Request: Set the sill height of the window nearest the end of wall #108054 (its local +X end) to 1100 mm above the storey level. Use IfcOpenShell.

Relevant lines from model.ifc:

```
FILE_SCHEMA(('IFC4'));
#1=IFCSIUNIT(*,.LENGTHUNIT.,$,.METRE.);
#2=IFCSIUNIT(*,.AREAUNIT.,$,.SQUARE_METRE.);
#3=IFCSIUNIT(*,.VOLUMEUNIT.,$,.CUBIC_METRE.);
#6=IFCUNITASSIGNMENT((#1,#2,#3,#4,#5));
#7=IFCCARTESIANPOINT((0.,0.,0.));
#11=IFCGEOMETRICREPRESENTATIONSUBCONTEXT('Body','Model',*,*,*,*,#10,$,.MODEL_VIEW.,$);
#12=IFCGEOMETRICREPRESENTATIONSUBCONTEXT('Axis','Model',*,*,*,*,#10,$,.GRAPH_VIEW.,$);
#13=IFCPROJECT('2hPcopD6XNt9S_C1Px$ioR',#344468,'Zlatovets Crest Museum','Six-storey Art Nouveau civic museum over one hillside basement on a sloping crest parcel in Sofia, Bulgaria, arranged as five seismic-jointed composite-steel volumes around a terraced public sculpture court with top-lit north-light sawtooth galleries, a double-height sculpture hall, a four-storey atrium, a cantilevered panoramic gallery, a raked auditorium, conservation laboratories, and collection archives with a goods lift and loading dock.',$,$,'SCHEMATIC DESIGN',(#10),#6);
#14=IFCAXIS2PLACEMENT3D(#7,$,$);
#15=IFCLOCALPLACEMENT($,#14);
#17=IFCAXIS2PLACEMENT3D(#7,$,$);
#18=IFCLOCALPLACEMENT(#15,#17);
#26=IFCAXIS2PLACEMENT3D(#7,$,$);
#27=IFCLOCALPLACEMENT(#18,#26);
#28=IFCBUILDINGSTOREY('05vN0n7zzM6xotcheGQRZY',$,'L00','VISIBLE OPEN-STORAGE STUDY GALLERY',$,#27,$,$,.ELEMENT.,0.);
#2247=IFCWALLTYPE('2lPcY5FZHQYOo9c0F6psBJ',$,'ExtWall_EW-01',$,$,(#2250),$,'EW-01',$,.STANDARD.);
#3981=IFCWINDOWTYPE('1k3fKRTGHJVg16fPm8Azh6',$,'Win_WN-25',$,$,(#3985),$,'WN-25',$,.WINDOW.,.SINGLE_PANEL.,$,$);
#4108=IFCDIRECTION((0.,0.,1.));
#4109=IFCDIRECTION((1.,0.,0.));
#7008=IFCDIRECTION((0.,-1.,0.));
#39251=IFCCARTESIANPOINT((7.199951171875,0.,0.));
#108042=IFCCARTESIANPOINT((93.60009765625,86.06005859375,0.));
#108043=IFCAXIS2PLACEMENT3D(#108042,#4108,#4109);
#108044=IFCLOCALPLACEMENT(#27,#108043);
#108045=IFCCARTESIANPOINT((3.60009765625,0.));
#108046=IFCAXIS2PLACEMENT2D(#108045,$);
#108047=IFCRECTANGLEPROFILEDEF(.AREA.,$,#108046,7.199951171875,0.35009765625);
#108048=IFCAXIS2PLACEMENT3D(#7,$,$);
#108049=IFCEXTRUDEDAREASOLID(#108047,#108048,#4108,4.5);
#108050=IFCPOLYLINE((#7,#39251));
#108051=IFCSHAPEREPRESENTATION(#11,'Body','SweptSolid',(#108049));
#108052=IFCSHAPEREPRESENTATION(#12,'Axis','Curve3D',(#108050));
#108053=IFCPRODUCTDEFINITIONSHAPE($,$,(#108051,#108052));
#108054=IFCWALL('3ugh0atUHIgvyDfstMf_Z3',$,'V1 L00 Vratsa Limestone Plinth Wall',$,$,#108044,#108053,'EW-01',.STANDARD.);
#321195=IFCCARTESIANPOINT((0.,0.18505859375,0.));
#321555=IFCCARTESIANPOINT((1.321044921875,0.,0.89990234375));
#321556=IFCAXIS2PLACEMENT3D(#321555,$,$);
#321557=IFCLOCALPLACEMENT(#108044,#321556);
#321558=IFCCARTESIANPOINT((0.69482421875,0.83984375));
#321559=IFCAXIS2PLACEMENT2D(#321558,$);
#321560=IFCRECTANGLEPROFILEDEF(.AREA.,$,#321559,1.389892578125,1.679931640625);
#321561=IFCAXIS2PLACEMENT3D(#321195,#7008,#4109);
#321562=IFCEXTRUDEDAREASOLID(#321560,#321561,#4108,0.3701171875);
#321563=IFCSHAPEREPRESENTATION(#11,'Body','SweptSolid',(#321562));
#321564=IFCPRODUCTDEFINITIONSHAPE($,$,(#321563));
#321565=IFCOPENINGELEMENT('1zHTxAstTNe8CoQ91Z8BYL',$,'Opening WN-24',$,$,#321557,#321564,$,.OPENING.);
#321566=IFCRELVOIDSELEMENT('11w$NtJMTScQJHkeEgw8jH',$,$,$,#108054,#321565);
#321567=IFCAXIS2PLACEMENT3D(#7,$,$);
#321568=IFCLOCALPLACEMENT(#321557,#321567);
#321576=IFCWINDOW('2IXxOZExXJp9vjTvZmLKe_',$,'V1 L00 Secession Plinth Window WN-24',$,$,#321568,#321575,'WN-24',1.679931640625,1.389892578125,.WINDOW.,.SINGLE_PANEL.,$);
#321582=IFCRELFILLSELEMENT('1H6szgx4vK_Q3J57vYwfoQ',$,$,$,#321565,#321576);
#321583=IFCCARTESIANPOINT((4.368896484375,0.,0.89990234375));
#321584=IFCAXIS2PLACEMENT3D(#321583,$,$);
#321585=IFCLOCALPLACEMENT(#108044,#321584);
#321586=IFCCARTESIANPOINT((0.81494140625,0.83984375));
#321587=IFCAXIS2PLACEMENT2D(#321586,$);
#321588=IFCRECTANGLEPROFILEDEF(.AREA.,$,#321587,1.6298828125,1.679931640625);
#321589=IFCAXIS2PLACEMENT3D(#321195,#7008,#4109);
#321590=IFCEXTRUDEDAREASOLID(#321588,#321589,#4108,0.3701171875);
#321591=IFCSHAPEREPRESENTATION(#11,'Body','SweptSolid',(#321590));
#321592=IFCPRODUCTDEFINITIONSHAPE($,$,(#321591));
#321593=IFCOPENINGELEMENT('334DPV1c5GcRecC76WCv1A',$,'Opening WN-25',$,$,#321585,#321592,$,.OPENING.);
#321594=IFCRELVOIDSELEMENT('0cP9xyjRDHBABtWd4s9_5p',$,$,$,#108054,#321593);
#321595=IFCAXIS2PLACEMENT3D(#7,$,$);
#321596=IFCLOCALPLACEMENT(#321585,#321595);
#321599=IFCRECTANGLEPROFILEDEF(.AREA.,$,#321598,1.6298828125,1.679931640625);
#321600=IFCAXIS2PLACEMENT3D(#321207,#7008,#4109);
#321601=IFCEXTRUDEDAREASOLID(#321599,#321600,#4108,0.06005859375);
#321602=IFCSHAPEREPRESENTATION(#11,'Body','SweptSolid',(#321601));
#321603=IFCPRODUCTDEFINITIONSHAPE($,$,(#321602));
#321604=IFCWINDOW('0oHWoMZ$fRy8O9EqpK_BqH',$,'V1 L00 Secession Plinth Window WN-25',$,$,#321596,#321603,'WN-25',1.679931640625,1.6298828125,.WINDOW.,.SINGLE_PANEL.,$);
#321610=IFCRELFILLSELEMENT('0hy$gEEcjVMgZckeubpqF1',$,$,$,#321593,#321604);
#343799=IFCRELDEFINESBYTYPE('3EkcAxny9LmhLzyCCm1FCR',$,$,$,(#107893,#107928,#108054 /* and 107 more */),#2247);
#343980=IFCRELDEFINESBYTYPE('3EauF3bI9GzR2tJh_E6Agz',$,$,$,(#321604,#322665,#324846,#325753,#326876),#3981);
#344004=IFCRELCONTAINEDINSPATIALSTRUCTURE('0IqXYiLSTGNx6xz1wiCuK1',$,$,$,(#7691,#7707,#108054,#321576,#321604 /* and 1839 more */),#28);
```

```python
import numpy as np
import ifcopenshell
import ifcopenshell.api.geometry
import ifcopenshell.geom
import ifcopenshell.util.element
import ifcopenshell.util.placement
import ifcopenshell.util.shape
import ifcopenshell.util.unit

model = ifcopenshell.open("model.ifc")
unit_scale = ifcopenshell.util.unit.calculate_unit_scale(model)

window = model.by_id(321604)
opening = window.FillsVoids[0].RelatingOpeningElement
storey = ifcopenshell.util.element.get_container(window, ifc_class="IfcBuildingStorey")
level = ifcopenshell.util.placement.get_local_placement(storey.ObjectPlacement)[2, 3]

# The opening's origin need not be at the sill, so measure its lowest point.
shape = ifcopenshell.geom.create_shape(ifcopenshell.geom.settings(), opening)
bottom = ifcopenshell.util.shape.get_shape_bottom_elevation(shape, shape.geometry) / unit_scale
dz = level + 1.1 - bottom

shift = np.array([0.0, 0.0, dz])
# The window is placed relative to its opening, so it follows when the opening moves.
matrix = ifcopenshell.util.placement.get_local_placement(opening.ObjectPlacement)
matrix[:3, 3] += shift
ifcopenshell.api.geometry.edit_object_placement(
    model, product=opening, matrix=matrix, is_si=False, should_transform_children=True
)

print(f"moved by {dz * unit_scale:+.3f} m")

model.write("model_edited.ifc")
```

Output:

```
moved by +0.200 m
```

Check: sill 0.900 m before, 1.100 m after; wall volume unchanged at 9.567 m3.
